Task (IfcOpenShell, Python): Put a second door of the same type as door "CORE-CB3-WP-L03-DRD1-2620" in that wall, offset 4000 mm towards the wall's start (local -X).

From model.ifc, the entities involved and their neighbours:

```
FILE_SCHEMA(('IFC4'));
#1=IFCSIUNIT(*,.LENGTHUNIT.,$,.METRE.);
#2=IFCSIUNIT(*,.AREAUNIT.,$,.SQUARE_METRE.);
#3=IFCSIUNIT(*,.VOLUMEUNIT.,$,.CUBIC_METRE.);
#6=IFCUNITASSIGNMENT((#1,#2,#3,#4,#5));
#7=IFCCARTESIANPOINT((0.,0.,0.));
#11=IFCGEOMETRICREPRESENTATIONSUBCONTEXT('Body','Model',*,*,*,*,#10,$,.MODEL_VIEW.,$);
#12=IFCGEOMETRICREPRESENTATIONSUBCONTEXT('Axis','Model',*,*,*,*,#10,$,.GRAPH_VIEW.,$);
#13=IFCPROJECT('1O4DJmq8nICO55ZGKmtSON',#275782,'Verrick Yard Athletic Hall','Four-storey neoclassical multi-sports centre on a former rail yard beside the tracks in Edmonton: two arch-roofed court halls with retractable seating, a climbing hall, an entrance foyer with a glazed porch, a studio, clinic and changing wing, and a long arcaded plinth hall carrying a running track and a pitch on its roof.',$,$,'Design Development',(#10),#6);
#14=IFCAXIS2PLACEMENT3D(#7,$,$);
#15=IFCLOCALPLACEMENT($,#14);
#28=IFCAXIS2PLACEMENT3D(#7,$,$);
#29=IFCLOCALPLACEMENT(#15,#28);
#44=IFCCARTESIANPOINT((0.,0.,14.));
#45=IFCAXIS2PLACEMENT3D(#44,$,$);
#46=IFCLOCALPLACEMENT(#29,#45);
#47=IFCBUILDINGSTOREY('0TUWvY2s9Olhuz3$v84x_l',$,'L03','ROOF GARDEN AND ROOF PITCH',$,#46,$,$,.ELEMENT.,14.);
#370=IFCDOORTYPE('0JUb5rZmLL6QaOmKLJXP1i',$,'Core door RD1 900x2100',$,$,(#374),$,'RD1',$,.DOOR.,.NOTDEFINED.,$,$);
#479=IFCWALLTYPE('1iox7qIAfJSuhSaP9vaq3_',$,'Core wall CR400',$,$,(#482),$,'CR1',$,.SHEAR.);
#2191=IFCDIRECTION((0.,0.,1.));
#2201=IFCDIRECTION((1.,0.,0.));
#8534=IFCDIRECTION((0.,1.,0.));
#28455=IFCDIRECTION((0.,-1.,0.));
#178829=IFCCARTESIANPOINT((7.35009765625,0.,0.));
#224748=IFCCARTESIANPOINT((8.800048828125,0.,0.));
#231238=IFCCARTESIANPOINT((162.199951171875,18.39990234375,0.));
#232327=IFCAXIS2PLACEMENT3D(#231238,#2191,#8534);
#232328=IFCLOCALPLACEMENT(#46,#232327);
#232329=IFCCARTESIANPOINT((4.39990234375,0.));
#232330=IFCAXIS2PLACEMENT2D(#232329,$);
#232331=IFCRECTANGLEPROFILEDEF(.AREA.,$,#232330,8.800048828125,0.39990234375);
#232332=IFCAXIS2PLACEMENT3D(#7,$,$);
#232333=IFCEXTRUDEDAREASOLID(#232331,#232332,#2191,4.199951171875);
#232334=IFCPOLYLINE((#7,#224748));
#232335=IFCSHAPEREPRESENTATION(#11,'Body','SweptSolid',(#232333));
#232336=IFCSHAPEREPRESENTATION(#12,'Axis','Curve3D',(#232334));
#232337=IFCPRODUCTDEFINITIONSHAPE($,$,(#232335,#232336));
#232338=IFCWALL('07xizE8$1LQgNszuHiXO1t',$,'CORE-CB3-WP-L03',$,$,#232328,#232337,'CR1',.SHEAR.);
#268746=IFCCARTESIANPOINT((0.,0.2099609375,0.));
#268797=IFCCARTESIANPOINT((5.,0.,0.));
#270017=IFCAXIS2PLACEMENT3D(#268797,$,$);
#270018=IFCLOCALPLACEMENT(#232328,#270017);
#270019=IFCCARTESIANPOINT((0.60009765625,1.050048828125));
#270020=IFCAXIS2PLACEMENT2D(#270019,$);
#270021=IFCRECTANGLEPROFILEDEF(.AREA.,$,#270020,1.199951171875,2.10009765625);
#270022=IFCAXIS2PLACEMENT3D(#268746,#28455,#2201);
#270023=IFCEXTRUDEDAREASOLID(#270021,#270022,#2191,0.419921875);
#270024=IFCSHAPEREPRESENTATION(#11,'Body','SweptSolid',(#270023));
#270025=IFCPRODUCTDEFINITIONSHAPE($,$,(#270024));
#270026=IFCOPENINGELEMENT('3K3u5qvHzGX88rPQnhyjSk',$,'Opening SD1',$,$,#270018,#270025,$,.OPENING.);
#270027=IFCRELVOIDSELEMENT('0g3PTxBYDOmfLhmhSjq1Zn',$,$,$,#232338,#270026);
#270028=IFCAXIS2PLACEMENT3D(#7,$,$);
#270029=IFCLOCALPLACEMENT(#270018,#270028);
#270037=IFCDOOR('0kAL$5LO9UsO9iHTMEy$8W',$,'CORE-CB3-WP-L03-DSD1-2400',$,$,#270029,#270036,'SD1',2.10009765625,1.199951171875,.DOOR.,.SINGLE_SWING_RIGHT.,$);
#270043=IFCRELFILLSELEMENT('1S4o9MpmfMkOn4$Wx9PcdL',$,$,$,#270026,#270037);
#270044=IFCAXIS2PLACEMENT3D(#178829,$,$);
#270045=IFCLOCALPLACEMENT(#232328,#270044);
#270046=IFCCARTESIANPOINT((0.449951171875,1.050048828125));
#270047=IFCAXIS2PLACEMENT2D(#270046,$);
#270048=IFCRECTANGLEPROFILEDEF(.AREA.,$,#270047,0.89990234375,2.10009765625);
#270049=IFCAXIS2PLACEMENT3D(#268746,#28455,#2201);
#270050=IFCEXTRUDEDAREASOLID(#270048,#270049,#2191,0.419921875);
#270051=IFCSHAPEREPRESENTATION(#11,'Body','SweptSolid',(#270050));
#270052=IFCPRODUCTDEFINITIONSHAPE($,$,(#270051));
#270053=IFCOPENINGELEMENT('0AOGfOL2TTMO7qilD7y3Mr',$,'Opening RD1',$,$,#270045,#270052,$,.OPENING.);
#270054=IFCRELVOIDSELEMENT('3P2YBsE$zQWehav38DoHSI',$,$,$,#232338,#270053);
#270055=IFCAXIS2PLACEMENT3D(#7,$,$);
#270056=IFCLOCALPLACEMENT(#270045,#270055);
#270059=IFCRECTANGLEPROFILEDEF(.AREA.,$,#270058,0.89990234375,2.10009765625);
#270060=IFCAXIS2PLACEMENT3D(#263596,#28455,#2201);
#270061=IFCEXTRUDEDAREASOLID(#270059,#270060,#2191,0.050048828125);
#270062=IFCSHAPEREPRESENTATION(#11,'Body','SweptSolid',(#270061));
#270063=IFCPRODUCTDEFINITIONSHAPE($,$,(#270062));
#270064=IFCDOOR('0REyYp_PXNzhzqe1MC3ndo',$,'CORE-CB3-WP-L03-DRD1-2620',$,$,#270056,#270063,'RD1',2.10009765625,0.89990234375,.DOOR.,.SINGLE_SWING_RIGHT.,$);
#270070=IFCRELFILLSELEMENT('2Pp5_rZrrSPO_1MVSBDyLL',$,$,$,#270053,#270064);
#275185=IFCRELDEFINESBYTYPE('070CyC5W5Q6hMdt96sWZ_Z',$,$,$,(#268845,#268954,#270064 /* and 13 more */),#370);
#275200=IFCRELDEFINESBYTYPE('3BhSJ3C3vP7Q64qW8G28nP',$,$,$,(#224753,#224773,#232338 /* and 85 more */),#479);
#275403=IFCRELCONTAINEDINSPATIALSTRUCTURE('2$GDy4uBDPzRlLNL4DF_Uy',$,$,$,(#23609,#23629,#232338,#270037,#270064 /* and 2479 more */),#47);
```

```python
import ifcopenshell
import ifcopenshell.api.feature
import ifcopenshell.api.geometry
import ifcopenshell.api.root
import ifcopenshell.geom
import ifcopenshell.util.element
import ifcopenshell.util.placement
import ifcopenshell.util.shape

model = ifcopenshell.open("model.ifc")
settings = ifcopenshell.geom.settings()


def volume(element):
    """Net volume in cubic metres, openings subtracted."""
    shape = ifcopenshell.geom.create_shape(settings, element)
    return ifcopenshell.util.shape.get_volume(shape.geometry)


door = model.by_id(270064)
opening = door.FillsVoids[0].RelatingOpeningElement
wall = opening.VoidsElements[0].RelatingBuildingElement
before = volume(wall)
shift = ifcopenshell.util.placement.get_local_placement(wall.ObjectPlacement)[:3, 0] * -4.0

# copy_class copies the void relationship, type, container and properties, but no geometry.
new_opening = ifcopenshell.api.root.copy_class(model, product=opening)
new_opening.Representation = ifcopenshell.util.element.copy_deep(
    model, opening.Representation, exclude=["IfcGeometricRepresentationContext", "IfcRepresentationMap"]
)
new_door = ifcopenshell.api.root.copy_class(model, product=door)
new_door.Representation = ifcopenshell.util.element.copy_deep(
    model, door.Representation, exclude=["IfcGeometricRepresentationContext", "IfcRepresentationMap"]
)
new_door.Tag = None
ifcopenshell.api.feature.add_filling(model, opening=new_opening, element=new_door)

for old, new in ((opening, new_opening), (door, new_door)):
    matrix = ifcopenshell.util.placement.get_local_placement(old.ObjectPlacement)
    matrix[:3, 3] += shift
    ifcopenshell.api.geometry.edit_object_placement(model, product=new, matrix=matrix, is_si=False)

after = volume(wall)

print(f"wall volume {before:.3f} -> {after:.3f} m3")

model.write("model_rev.ifc")
```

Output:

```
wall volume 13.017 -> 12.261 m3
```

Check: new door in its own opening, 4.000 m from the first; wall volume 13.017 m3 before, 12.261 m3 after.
